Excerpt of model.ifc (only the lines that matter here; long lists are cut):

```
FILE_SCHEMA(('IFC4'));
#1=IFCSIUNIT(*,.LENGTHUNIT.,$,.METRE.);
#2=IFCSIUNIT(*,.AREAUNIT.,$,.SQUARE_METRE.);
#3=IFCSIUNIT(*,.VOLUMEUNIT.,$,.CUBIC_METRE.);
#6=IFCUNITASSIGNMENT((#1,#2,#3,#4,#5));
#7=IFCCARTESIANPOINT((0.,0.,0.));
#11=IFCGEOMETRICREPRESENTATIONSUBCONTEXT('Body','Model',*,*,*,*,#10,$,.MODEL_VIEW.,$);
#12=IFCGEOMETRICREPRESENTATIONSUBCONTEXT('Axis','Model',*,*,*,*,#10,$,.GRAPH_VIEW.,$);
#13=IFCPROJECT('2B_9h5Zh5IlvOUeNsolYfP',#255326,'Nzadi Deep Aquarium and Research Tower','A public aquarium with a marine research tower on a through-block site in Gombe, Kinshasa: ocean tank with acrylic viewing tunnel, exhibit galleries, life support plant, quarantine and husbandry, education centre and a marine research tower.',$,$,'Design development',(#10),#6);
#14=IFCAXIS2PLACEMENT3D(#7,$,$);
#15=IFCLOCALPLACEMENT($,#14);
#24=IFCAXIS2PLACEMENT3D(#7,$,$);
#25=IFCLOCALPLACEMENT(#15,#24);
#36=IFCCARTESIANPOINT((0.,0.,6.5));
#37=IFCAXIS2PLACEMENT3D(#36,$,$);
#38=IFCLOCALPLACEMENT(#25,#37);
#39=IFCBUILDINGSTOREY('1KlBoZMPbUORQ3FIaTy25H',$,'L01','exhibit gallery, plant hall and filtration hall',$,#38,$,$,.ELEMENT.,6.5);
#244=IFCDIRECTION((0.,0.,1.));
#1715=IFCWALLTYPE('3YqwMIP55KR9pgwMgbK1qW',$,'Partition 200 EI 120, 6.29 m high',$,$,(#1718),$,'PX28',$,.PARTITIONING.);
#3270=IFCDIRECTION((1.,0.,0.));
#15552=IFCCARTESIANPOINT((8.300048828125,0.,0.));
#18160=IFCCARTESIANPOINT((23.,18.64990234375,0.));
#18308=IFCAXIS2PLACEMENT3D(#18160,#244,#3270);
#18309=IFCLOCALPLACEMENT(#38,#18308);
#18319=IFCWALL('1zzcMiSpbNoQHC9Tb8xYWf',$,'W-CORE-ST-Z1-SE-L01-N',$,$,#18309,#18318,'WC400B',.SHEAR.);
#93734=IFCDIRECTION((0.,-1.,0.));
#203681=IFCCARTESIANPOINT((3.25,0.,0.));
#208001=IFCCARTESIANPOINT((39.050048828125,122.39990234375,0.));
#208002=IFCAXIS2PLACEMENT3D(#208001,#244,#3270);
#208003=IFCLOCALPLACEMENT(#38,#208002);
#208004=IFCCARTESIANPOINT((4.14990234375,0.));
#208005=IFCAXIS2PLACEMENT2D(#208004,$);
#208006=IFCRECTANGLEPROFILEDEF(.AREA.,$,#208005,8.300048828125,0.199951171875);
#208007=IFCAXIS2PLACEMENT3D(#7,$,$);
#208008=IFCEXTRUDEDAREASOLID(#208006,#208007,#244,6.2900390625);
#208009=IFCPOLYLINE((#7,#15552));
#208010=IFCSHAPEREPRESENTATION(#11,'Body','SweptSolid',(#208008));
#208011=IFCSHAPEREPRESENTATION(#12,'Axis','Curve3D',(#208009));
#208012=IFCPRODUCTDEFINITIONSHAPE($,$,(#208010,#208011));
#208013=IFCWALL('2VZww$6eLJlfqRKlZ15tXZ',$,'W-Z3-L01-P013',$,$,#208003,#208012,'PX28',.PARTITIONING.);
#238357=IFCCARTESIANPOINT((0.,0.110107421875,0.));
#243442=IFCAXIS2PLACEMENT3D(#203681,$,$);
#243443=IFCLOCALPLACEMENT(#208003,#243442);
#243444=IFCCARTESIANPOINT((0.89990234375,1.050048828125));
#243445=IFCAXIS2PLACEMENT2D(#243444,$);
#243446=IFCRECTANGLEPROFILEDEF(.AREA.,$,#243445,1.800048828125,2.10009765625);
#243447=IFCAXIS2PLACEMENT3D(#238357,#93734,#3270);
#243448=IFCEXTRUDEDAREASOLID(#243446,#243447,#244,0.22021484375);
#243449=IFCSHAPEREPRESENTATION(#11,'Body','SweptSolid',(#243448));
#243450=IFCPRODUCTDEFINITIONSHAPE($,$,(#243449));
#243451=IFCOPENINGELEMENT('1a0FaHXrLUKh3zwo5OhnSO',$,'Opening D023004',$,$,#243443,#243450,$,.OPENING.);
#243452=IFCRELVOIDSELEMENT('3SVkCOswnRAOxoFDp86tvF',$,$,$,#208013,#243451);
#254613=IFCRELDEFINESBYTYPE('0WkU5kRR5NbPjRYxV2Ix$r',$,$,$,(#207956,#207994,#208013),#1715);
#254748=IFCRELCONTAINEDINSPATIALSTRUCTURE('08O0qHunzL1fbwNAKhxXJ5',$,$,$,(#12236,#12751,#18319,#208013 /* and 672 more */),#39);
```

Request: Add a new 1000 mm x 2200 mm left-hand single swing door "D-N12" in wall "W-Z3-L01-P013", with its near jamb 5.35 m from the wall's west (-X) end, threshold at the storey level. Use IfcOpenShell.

```python
import numpy as np
import ifcopenshell
import ifcopenshell.api.feature
import ifcopenshell.api.geometry
import ifcopenshell.api.root
import ifcopenshell.api.spatial
import ifcopenshell.geom
import ifcopenshell.util.element
import ifcopenshell.util.placement
import ifcopenshell.util.representation
import ifcopenshell.util.shape
import ifcopenshell.util.unit

model = ifcopenshell.open("model.ifc")
unit_scale = ifcopenshell.util.unit.calculate_unit_scale(model)
settings = ifcopenshell.geom.settings()


def volume(element):
    """Net volume in cubic metres, openings subtracted."""
    shape = ifcopenshell.geom.create_shape(settings, element)
    return ifcopenshell.util.shape.get_volume(shape.geometry)


wall = model.by_guid("2VZww$6eLJlfqRKlZ15tXZ")
storey = ifcopenshell.util.element.get_container(wall, ifc_class="IfcBuildingStorey")
context = ifcopenshell.util.representation.get_context(model, "Model", "Body", "MODEL_VIEW")
before = volume(wall)

width, height, from_end, sill = 1, 2.2, 5.35, 0.0  # metres

# The wall runs along its own X axis, and the end named is its -X end.
wall_shape = ifcopenshell.geom.create_shape(settings, wall)
x, y, z = ifcopenshell.util.shape.get_vertices(wall_shape.geometry).T
start = x.min() + from_end
face, thickness = float(y.min()), float(y.max() - y.min())
wall_matrix = ifcopenshell.util.placement.get_local_placement(wall.ObjectPlacement)
level = ifcopenshell.util.placement.get_local_placement(storey.ObjectPlacement)[2, 3]


def in_wall(x, y):
    """Placement at x, y metres in the wall's axes, at sill height."""
    matrix = wall_matrix.copy()
    matrix[:, 3] = wall_matrix @ np.array([x / unit_scale, y / unit_scale, 0.0, 1.0])
    matrix[2, 3] = level + sill / unit_scale
    return matrix


# Opening: a box that overshoots both wall faces by 50 mm.
opening = ifcopenshell.api.root.create_entity(model, ifc_class="IfcOpeningElement", predefined_type="OPENING")
box = ifcopenshell.api.geometry.add_wall_representation(
    model, context=context, length=width, height=height, thickness=thickness + 0.1
)
ifcopenshell.api.geometry.assign_representation(model, product=opening, representation=box)
ifcopenshell.api.geometry.edit_object_placement(model, product=opening, matrix=in_wall(start, face - 0.05), is_si=False)
ifcopenshell.api.feature.add_feature(model, feature=opening, element=wall)

door = ifcopenshell.api.root.create_entity(model, ifc_class="IfcDoor", name="D-N12", predefined_type="DOOR")
door.OverallWidth, door.OverallHeight = width / unit_scale, height / unit_scale
door.OperationType = "SINGLE_SWING_LEFT"
body = ifcopenshell.api.geometry.add_door_representation(
    model,
    context=context,
    overall_width=door.OverallWidth,
    overall_height=door.OverallHeight,
    operation_type="SINGLE_SWING_LEFT",
    lining_properties={"LiningDepth": thickness / unit_scale, "ThresholdDepth": thickness / unit_scale},
)
ifcopenshell.api.geometry.assign_representation(model, product=door, representation=body)
ifcopenshell.api.spatial.assign_container(model, products=[door], relating_structure=storey)
ifcopenshell.api.feature.add_filling(model, opening=opening, element=door)

# The lining spans the wall, so the door starts at the wall face.
ifcopenshell.api.geometry.edit_object_placement(model, product=door, matrix=in_wall(start, face), is_si=False)

after = volume(wall)

print(f"wall volume {before:.3f} -> {after:.3f} m3")

model.write("model_rev.ifc")
```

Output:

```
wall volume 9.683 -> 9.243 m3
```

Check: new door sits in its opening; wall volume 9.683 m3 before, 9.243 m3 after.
